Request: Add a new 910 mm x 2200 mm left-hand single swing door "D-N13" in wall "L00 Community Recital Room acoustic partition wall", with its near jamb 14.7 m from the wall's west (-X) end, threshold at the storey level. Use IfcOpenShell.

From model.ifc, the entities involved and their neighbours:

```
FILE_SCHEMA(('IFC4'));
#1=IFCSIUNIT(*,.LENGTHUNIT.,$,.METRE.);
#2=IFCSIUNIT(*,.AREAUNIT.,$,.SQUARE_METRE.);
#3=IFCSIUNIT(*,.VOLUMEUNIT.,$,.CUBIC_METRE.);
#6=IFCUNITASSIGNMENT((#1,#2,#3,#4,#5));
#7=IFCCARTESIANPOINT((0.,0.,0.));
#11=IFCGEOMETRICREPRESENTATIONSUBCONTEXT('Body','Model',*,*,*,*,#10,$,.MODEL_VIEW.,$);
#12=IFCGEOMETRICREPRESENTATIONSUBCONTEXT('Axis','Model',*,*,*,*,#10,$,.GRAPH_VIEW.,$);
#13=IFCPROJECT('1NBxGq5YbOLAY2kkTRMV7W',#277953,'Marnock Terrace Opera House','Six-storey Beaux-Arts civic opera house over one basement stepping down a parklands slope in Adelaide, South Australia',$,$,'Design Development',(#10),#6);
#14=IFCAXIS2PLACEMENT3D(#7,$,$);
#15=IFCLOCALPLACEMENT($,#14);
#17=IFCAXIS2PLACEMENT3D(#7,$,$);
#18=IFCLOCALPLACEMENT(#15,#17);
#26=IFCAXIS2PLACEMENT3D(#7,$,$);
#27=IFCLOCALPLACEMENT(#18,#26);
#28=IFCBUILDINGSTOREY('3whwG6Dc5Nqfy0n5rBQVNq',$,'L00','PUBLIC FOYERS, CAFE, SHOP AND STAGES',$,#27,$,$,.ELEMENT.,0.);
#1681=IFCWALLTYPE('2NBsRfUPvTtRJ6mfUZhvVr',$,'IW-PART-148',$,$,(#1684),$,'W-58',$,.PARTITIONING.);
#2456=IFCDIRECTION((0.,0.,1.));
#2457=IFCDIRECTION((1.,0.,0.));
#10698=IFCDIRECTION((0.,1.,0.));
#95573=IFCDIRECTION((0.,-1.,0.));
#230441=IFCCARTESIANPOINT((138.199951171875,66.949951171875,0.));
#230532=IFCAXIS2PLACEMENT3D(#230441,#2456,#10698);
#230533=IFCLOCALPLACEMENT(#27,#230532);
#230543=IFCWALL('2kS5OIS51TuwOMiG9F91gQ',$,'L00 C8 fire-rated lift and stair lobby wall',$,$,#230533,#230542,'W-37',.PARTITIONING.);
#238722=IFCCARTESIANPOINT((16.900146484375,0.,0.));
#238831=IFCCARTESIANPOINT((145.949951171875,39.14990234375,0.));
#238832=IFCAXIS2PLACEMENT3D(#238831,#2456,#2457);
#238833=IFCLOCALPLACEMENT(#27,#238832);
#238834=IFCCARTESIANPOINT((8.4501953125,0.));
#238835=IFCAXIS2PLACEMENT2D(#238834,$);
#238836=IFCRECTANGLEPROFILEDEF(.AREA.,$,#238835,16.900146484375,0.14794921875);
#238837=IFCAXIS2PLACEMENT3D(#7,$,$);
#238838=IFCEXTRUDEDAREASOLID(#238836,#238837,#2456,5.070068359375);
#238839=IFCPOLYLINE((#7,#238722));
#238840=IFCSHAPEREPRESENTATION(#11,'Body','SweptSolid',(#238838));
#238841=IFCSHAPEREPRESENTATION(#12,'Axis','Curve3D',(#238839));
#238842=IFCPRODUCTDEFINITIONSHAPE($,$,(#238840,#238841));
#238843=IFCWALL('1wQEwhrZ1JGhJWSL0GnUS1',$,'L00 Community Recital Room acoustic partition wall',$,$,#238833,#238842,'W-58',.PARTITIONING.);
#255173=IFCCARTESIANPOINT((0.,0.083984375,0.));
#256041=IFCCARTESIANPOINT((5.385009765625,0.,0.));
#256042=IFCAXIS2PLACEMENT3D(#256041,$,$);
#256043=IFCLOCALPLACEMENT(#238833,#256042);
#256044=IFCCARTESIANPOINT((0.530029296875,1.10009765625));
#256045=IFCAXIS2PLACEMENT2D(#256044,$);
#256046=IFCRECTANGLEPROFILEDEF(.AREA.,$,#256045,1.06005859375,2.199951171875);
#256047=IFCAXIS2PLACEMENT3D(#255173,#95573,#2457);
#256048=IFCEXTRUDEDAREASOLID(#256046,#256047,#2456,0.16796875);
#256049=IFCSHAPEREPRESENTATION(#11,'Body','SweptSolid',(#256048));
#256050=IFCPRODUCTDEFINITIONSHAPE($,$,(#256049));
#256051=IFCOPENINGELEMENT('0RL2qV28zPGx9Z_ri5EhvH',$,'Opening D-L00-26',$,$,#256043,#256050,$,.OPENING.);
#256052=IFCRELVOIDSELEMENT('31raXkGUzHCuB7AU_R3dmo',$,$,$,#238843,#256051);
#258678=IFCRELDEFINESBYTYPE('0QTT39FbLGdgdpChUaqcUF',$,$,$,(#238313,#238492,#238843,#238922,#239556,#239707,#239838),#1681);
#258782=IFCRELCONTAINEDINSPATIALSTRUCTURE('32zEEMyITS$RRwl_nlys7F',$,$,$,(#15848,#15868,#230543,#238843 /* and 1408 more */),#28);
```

```python
import numpy as np
import ifcopenshell
import ifcopenshell.api.feature
import ifcopenshell.api.geometry
import ifcopenshell.api.root
import ifcopenshell.api.spatial
import ifcopenshell.geom
import ifcopenshell.util.element
import ifcopenshell.util.placement
import ifcopenshell.util.representation
import ifcopenshell.util.shape
import ifcopenshell.util.unit

model = ifcopenshell.open("model.ifc")
unit_scale = ifcopenshell.util.unit.calculate_unit_scale(model)
settings = ifcopenshell.geom.settings()


def volume(element):
    """Net volume in cubic metres, openings subtracted."""
    shape = ifcopenshell.geom.create_shape(settings, element)
    return ifcopenshell.util.shape.get_volume(shape.geometry)


wall = model.by_guid("1wQEwhrZ1JGhJWSL0GnUS1")
storey = ifcopenshell.util.element.get_container(wall, ifc_class="IfcBuildingStorey")
context = ifcopenshell.util.representation.get_context(model, "Model", "Body", "MODEL_VIEW")
before = volume(wall)

width, height, from_end, sill = 0.91, 2.2, 14.7, 0.0  # metres

# The wall runs along its own X axis, and the end named is its -X end.
wall_shape = ifcopenshell.geom.create_shape(settings, wall)
x, y, z = ifcopenshell.util.shape.get_vertices(wall_shape.geometry).T
start = x.min() + from_end
face, thickness = float(y.min()), float(y.max() - y.min())
wall_matrix = ifcopenshell.util.placement.get_local_placement(wall.ObjectPlacement)
level = ifcopenshell.util.placement.get_local_placement(storey.ObjectPlacement)[2, 3]


def in_wall(x, y):
    """Placement at x, y metres in the wall's axes, at sill height."""
    matrix = wall_matrix.copy()
    matrix[:, 3] = wall_matrix @ np.array([x / unit_scale, y / unit_scale, 0.0, 1.0])
    matrix[2, 3] = level + sill / unit_scale
    return matrix


# Opening: a box that overshoots both wall faces by 50 mm.
opening = ifcopenshell.api.root.create_entity(model, ifc_class="IfcOpeningElement", predefined_type="OPENING")
box = ifcopenshell.api.geometry.add_wall_representation(
    model, context=context, length=width, height=height, thickness=thickness + 0.1
)
ifcopenshell.api.geometry.assign_representation(model, product=opening, representation=box)
ifcopenshell.api.geometry.edit_object_placement(model, product=opening, matrix=in_wall(start, face - 0.05), is_si=False)
ifcopenshell.api.feature.add_feature(model, feature=opening, element=wall)

door = ifcopenshell.api.root.create_entity(model, ifc_class="IfcDoor", name="D-N13", predefined_type="DOOR")
door.OverallWidth, door.OverallHeight = width / unit_scale, height / unit_scale
door.OperationType = "SINGLE_SWING_LEFT"
body = ifcopenshell.api.geometry.add_door_representation(
    model,
    context=context,
    overall_width=door.OverallWidth,
    overall_height=door.OverallHeight,
    operation_type="SINGLE_SWING_LEFT",
    lining_properties={"LiningDepth": thickness / unit_scale, "ThresholdDepth": thickness / unit_scale},
)
ifcopenshell.api.geometry.assign_representation(model, product=door, representation=body)
ifcopenshell.api.spatial.assign_container(model, products=[door], relating_structure=storey)
ifcopenshell.api.feature.add_filling(model, opening=opening, element=door)

# The lining spans the wall, so the door starts at the wall face.
ifcopenshell.api.geometry.edit_object_placement(model, product=door, matrix=in_wall(start, face), is_si=False)

after = volume(wall)

print(f"wall volume {before:.3f} -> {after:.3f} m3")

model.write("model_updated.ifc")
```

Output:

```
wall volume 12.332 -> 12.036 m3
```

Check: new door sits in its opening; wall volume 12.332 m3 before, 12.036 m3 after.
